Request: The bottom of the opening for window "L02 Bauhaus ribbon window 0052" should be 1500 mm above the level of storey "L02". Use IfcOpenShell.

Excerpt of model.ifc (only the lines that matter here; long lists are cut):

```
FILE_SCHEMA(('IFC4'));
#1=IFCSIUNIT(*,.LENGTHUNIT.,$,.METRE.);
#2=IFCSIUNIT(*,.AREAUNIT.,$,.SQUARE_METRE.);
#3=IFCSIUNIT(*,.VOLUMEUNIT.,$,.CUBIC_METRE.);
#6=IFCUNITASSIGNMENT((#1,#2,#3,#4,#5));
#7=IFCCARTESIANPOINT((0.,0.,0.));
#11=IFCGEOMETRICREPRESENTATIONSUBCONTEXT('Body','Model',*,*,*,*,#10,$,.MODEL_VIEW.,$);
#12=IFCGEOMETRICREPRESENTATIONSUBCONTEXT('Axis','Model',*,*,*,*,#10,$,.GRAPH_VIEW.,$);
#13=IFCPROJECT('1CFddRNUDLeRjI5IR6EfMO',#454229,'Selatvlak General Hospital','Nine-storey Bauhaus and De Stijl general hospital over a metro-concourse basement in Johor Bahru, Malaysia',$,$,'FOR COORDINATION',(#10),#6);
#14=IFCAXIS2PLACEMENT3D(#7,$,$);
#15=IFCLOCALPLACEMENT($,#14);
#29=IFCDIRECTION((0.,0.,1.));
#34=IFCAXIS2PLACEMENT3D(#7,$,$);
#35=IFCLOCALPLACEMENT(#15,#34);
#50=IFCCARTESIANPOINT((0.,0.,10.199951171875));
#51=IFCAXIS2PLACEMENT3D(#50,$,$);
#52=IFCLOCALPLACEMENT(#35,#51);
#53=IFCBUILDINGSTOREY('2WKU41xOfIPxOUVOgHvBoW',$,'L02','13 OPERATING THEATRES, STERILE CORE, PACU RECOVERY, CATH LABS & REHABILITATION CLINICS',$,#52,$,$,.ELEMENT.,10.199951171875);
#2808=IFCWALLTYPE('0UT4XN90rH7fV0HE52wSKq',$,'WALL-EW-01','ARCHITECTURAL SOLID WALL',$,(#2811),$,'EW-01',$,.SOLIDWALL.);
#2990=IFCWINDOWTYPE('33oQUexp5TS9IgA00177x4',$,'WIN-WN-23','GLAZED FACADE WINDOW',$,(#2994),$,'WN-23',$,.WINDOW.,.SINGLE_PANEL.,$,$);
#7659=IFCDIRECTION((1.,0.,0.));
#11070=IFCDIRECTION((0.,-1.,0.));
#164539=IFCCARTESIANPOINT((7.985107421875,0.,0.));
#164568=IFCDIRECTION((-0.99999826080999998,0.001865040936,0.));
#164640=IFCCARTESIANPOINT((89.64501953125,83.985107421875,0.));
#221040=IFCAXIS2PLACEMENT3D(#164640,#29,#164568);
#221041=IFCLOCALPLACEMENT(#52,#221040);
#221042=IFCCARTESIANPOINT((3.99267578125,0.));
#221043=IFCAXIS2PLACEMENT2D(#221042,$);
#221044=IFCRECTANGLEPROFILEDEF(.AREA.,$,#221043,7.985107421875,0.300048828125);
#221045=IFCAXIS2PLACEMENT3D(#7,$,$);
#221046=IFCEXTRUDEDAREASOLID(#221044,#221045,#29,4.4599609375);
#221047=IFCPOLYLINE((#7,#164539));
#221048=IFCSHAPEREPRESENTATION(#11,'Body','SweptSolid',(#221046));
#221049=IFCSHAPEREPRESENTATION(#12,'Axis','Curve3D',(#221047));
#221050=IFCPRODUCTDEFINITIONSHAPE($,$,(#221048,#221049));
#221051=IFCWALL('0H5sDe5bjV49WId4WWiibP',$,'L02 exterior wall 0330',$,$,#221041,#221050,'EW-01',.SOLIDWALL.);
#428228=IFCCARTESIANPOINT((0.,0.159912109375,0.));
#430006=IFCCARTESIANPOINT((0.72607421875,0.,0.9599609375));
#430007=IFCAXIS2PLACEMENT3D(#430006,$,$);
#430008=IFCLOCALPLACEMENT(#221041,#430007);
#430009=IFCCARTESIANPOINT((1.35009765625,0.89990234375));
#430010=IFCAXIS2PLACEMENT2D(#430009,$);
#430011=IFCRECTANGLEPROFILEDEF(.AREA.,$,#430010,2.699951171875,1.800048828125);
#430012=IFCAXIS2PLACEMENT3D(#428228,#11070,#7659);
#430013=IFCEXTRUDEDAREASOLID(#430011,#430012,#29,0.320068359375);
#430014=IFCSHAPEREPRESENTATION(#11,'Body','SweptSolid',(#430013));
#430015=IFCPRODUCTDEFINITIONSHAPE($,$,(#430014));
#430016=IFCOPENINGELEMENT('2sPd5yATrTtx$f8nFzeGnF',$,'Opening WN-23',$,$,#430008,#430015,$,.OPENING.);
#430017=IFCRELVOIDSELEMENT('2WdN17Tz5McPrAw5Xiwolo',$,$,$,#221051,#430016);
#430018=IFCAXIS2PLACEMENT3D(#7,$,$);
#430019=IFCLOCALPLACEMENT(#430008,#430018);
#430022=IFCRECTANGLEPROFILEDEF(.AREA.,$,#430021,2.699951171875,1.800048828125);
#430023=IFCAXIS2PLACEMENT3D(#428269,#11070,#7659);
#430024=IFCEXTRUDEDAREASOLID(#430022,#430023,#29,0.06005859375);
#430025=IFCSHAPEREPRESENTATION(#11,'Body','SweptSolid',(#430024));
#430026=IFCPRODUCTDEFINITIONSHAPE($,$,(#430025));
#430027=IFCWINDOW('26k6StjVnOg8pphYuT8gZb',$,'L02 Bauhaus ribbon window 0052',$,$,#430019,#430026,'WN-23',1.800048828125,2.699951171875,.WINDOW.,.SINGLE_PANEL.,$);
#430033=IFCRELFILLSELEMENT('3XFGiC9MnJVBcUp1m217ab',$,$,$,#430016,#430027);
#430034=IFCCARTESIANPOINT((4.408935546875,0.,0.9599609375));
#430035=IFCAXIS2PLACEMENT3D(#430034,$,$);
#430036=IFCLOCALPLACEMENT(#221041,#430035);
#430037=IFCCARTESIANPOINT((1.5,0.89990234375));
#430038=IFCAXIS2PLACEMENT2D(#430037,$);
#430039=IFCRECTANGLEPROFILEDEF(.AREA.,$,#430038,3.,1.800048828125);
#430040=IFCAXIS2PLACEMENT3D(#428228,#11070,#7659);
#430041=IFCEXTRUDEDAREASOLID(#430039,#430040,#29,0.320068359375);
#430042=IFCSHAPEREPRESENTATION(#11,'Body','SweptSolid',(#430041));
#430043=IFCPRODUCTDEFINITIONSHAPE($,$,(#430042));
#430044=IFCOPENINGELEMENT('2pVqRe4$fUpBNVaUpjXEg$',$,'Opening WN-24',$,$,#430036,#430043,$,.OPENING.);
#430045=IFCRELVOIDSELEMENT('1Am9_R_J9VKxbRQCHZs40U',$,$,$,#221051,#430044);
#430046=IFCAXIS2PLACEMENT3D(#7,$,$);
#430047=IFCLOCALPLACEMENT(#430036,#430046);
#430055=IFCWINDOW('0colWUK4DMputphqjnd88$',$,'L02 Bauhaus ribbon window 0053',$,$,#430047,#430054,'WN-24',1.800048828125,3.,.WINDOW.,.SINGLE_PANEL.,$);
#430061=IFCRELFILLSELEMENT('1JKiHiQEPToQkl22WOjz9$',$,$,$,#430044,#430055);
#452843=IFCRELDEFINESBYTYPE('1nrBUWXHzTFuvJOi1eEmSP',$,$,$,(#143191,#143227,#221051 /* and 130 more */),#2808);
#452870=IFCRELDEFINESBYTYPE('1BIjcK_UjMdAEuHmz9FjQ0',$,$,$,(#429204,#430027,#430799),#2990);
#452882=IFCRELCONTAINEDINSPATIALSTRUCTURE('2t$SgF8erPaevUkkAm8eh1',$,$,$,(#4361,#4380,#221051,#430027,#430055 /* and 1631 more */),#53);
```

```python
import numpy as np
import ifcopenshell
import ifcopenshell.api.geometry
import ifcopenshell.geom
import ifcopenshell.util.element
import ifcopenshell.util.placement
import ifcopenshell.util.shape
import ifcopenshell.util.unit

model = ifcopenshell.open("model.ifc")
unit_scale = ifcopenshell.util.unit.calculate_unit_scale(model)

window = model.by_id(430027)
opening = window.FillsVoids[0].RelatingOpeningElement
storey = ifcopenshell.util.element.get_container(window, ifc_class="IfcBuildingStorey")
level = ifcopenshell.util.placement.get_local_placement(storey.ObjectPlacement)[2, 3]

# The opening's origin need not be at the sill, so measure its lowest point.
shape = ifcopenshell.geom.create_shape(ifcopenshell.geom.settings(), opening)
bottom = ifcopenshell.util.shape.get_shape_bottom_elevation(shape, shape.geometry) / unit_scale
dz = level + 1.5 / unit_scale - bottom

shift = np.array([0.0, 0.0, dz])
# The window is placed relative to its opening, so it follows when the opening moves.
matrix = ifcopenshell.util.placement.get_local_placement(opening.ObjectPlacement)
matrix[:3, 3] += shift
ifcopenshell.api.geometry.edit_object_placement(
    model, product=opening, matrix=matrix, is_si=False, should_transform_children=True
)

print(f"moved by {dz * unit_scale:+.3f} m")

model.write("model_v2.ifc")
```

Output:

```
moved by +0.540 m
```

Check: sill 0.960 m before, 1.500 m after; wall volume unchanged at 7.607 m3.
